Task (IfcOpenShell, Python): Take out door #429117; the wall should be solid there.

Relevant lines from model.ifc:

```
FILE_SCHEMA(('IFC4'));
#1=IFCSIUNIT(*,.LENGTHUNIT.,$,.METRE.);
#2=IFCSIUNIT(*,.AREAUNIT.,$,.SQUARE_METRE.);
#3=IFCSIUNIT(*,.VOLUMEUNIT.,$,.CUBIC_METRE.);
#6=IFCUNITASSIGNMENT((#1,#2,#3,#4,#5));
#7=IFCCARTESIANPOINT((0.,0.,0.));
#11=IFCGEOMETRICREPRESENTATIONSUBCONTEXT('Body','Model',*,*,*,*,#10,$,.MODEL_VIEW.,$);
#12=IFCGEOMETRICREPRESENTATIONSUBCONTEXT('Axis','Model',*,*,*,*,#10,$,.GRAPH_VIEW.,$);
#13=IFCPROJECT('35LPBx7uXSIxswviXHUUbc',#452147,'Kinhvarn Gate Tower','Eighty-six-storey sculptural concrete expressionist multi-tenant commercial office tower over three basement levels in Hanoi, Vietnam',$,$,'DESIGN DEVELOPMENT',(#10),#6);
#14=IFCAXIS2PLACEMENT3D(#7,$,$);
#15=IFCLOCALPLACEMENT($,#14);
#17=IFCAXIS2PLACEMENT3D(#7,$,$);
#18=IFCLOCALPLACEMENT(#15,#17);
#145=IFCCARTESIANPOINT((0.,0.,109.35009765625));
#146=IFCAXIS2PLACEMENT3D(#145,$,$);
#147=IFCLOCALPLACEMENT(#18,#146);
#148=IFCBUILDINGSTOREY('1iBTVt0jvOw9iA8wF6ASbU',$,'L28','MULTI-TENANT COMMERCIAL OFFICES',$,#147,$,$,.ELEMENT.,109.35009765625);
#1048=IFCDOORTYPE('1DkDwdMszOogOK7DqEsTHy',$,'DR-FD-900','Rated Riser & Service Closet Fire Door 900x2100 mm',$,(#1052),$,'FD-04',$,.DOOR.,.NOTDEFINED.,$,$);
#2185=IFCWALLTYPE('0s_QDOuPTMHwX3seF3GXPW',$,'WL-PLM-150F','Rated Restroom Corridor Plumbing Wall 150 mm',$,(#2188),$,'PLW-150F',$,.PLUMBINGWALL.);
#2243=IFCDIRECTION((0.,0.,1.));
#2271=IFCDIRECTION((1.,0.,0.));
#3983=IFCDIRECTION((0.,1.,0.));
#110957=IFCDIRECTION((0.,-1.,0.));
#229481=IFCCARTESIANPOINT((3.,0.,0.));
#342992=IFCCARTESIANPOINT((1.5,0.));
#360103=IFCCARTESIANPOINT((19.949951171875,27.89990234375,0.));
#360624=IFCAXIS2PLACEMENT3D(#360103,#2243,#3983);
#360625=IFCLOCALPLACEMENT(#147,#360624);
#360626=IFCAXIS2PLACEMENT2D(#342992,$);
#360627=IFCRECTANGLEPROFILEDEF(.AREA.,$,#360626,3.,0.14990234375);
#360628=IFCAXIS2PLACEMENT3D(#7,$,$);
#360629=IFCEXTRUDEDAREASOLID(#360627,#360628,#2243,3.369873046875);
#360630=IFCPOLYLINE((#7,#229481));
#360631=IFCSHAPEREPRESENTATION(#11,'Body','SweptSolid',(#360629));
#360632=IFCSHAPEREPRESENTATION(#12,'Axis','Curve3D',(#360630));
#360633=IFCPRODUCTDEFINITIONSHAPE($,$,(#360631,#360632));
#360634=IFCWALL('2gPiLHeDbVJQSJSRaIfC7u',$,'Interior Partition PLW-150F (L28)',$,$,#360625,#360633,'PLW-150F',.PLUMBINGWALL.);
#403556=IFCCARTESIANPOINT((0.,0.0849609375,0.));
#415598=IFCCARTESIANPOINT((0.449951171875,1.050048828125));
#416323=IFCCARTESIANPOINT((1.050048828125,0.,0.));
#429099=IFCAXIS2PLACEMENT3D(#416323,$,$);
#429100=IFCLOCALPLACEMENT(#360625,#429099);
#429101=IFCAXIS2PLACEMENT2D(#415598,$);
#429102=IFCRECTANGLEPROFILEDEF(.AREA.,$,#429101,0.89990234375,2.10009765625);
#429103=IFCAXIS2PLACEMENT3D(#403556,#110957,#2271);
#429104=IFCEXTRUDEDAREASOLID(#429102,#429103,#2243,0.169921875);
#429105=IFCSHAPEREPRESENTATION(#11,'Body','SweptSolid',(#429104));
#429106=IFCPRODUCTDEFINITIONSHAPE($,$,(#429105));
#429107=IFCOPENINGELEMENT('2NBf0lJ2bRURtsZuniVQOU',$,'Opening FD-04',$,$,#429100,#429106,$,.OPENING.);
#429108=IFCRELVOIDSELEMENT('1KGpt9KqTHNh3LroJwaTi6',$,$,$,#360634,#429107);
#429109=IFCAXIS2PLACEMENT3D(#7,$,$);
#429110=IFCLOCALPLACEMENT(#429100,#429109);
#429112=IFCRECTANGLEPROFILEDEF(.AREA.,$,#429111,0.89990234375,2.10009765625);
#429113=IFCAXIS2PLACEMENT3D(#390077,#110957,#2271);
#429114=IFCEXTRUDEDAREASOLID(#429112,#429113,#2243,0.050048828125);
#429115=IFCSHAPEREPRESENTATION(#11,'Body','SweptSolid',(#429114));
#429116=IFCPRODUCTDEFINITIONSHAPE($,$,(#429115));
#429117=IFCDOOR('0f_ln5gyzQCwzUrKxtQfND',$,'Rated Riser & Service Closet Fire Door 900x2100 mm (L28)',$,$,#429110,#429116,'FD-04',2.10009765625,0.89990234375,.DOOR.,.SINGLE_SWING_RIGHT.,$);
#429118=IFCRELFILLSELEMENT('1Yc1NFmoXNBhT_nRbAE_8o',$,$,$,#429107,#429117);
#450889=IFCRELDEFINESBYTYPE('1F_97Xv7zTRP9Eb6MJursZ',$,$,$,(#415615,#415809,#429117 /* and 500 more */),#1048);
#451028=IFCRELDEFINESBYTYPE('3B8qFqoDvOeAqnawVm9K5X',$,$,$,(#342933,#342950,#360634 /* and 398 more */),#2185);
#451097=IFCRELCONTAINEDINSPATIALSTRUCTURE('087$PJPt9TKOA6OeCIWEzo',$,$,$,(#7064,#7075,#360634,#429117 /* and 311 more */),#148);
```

```python
import ifcopenshell
import ifcopenshell.api.feature
import ifcopenshell.api.root
import ifcopenshell.geom
import ifcopenshell.util.shape

model = ifcopenshell.open("model.ifc")
settings = ifcopenshell.geom.settings()


def volume(element):
    """Net volume in cubic metres, openings subtracted."""
    shape = ifcopenshell.geom.create_shape(settings, element)
    return ifcopenshell.util.shape.get_volume(shape.geometry)


door = model.by_guid("0f_ln5gyzQCwzUrKxtQfND")
opening = door.FillsVoids[0].RelatingOpeningElement
wall = opening.VoidsElements[0].RelatingBuildingElement
before = volume(wall)

ifcopenshell.api.root.remove_product(model, product=door)
ifcopenshell.api.feature.remove_feature(model, feature=opening)

after = volume(wall)

print(f"wall volume {before:.3f} -> {after:.3f} m3")

model.write("model_updated.ifc")
```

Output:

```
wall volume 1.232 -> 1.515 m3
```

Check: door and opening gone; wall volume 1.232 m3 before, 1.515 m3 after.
